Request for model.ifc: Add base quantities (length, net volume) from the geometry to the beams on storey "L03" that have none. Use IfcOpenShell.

First a look at what the model holds.

```python
import ifcopenshell
import ifcopenshell.util.element
import ifcopenshell.util.unit

model = ifcopenshell.open("model.ifc")
print(model.schema)
for unit_type in ("LENGTHUNIT", "AREAUNIT", "VOLUMEUNIT"):
    print(unit_type, ifcopenshell.util.unit.calculate_unit_scale(model, unit_type))
storey = next(s for s in model.by_type("IfcBuildingStorey") if s.Name == "L03")
beams = [e for e in ifcopenshell.util.element.get_decomposition(storey) if e.is_a("IfcBeam")]
for e in sorted(beams, key=lambda e: e.id()):
    print(e.id(), e.is_a(), e.Name, list(ifcopenshell.util.element.get_psets(e, qtos_only=True)), sep=" | ")
```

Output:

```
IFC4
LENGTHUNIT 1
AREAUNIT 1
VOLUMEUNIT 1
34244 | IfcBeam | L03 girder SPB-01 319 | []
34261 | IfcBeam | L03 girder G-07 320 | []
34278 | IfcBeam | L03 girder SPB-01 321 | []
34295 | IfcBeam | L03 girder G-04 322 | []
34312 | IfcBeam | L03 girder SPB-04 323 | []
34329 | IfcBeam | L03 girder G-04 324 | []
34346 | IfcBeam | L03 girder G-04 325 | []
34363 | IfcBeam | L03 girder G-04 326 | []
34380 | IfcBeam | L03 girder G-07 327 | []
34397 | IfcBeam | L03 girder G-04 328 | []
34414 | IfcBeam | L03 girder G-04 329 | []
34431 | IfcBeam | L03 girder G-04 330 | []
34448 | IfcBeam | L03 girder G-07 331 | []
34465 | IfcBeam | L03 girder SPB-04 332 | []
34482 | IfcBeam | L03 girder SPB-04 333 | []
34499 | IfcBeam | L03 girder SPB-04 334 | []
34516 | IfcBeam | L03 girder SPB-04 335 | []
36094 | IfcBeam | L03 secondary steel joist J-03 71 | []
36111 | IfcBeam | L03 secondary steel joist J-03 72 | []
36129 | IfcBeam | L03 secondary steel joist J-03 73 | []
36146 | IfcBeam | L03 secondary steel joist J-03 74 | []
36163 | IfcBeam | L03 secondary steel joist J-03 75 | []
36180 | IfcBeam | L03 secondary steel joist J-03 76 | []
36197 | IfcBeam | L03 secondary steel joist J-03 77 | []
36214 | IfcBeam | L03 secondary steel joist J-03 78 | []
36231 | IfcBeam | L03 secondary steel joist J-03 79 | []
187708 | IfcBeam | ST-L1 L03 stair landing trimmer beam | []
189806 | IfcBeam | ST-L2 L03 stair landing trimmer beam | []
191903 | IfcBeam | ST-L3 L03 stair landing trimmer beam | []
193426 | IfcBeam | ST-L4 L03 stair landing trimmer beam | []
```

```python
import ifcopenshell
import ifcopenshell.api.pset
import ifcopenshell.geom
import ifcopenshell.util.element
import ifcopenshell.util.shape
import ifcopenshell.util.unit

model = ifcopenshell.open("model.ifc")
unit_scale = ifcopenshell.util.unit.calculate_unit_scale(model)
volume_scale = ifcopenshell.util.unit.calculate_unit_scale(model, "VOLUMEUNIT")
settings = ifcopenshell.geom.settings()

storey = next(s for s in model.by_type("IfcBuildingStorey") if s.Name == "L03")
beams = [e for e in ifcopenshell.util.element.get_decomposition(storey) if e.is_a("IfcBeam")]

for e in sorted(beams, key=lambda e: e.id()):
    if ifcopenshell.util.element.get_psets(e, qtos_only=True, should_inherit=False):
        continue
    # Geometry comes back in metres, in the element's own axes.
    shape = ifcopenshell.geom.create_shape(settings, e)
    values = {
        "Length": ifcopenshell.util.shape.get_max_xyz(shape.geometry) / unit_scale,
        "NetVolume": ifcopenshell.util.shape.get_volume(shape.geometry) / volume_scale,
    }
    qto = ifcopenshell.api.pset.add_qto(model, product=e, name="Qto_BeamBaseQuantities")
    ifcopenshell.api.pset.edit_qto(model, qto=qto, properties=values)
    print(e.id(), {k: round(v, 3) for k, v in values.items()})

model.write("model-out.ifc")
```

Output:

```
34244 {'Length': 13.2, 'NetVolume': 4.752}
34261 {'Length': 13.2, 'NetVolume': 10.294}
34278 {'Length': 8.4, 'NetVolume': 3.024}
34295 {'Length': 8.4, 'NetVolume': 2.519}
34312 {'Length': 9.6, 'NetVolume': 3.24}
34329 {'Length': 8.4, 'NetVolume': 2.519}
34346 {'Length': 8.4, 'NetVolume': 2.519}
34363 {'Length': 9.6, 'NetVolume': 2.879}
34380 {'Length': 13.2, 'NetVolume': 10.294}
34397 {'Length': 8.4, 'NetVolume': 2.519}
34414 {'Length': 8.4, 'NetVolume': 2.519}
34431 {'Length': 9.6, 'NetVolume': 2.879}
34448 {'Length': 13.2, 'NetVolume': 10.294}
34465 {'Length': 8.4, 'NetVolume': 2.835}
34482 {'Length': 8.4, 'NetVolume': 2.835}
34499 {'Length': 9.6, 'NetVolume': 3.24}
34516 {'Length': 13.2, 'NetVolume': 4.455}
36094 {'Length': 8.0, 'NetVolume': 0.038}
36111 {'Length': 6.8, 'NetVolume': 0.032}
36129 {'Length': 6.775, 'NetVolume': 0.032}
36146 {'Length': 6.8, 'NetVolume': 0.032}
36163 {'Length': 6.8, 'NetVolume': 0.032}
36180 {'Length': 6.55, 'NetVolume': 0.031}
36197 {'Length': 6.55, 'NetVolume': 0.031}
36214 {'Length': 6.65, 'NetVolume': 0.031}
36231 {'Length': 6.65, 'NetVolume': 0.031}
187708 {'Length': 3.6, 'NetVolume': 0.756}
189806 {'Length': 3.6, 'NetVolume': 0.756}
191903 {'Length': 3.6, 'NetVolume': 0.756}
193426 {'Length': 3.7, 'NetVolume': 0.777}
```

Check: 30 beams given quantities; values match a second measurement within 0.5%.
